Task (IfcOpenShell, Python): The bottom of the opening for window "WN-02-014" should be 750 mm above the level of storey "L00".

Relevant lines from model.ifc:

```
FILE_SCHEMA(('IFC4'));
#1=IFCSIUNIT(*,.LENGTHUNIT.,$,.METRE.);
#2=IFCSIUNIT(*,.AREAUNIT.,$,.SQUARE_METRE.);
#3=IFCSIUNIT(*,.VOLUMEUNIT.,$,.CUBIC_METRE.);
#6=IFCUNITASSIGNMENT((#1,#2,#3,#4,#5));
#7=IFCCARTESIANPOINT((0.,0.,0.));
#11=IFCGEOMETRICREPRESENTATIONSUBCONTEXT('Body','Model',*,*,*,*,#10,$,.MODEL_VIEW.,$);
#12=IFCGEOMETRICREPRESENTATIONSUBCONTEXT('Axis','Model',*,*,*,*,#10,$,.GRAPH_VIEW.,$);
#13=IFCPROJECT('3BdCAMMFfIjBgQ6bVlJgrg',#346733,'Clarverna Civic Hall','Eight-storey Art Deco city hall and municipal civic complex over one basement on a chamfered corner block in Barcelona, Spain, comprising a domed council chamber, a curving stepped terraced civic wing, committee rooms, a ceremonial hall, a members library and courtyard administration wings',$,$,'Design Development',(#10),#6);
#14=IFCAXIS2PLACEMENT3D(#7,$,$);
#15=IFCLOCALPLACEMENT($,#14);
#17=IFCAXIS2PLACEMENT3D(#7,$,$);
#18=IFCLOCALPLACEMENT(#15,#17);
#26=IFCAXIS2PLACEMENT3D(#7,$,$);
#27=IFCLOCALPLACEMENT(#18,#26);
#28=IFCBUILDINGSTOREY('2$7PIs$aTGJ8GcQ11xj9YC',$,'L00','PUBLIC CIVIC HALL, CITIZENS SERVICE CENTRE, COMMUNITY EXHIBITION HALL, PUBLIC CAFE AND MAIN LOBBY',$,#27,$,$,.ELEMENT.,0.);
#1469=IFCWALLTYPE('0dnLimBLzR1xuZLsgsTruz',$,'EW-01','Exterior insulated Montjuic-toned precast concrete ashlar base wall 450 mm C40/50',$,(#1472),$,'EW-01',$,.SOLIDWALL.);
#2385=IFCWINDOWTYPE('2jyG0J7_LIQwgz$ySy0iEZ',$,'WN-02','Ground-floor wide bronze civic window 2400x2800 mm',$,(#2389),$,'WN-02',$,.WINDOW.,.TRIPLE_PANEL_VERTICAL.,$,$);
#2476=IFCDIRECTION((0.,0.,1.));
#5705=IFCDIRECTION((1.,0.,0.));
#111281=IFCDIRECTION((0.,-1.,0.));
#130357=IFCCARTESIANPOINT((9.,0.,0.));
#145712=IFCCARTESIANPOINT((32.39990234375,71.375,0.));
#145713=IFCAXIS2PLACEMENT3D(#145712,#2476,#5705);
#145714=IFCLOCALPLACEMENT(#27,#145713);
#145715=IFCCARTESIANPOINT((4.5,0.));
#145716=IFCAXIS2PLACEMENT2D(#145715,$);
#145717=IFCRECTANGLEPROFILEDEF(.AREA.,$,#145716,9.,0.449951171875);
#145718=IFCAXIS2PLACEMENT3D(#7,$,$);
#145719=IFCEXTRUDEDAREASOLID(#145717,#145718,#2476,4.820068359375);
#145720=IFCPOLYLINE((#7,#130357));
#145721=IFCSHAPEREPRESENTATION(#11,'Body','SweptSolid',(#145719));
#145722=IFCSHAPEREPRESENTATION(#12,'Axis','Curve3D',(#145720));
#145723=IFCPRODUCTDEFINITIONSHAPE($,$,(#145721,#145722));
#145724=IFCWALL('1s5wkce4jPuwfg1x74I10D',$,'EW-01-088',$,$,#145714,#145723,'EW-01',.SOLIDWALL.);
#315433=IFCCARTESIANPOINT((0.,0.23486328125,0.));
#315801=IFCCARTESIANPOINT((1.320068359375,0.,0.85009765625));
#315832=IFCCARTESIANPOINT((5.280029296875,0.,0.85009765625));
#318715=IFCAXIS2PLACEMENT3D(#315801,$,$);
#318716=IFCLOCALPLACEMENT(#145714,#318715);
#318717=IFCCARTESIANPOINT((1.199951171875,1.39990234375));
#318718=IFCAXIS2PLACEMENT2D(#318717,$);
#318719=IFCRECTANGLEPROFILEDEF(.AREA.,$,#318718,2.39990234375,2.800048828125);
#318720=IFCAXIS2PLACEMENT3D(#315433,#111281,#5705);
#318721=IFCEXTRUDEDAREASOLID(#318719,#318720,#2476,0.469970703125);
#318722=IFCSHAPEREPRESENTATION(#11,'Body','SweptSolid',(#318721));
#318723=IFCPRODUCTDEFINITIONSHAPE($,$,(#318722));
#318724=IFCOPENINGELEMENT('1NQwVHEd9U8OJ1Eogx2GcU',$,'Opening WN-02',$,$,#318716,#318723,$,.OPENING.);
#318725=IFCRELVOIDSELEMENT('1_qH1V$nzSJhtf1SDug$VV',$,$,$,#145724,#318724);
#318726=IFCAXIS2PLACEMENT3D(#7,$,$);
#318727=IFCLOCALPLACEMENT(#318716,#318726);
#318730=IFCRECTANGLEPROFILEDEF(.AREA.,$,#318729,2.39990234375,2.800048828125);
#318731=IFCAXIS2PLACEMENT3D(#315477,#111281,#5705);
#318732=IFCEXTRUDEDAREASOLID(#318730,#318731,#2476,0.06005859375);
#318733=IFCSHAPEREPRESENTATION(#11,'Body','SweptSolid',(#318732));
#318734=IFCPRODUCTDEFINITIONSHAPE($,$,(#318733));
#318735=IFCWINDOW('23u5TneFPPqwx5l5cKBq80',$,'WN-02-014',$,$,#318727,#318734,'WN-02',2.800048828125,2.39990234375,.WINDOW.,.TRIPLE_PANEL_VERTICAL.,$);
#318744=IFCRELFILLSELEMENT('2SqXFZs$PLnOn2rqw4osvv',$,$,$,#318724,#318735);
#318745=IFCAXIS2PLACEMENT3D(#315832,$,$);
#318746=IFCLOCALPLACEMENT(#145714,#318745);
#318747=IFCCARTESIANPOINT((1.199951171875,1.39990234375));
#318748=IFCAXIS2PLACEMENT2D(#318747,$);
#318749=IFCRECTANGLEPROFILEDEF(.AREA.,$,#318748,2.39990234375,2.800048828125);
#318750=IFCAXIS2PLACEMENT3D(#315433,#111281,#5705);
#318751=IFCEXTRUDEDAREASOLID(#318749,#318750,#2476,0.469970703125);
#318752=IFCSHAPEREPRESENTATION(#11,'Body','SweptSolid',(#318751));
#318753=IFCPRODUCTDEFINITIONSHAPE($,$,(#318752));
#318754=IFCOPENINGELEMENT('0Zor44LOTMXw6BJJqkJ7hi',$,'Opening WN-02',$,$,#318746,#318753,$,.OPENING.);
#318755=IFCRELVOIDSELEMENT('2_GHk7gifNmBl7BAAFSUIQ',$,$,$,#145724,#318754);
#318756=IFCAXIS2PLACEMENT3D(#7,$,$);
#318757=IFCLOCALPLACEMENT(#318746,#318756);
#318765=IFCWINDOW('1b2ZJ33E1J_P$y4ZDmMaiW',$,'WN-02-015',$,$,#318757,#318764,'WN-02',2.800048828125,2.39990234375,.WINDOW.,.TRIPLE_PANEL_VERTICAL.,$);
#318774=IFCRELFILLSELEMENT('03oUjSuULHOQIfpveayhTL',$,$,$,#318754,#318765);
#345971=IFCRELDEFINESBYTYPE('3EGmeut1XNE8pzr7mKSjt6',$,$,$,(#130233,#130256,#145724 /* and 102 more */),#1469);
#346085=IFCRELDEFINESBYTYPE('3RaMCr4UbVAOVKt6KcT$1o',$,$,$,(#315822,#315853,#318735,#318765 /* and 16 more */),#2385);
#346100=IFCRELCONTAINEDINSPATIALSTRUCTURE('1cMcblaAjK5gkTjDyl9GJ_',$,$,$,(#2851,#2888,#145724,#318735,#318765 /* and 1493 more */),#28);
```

```python
import numpy as np
import ifcopenshell
import ifcopenshell.api.geometry
import ifcopenshell.geom
import ifcopenshell.util.element
import ifcopenshell.util.placement
import ifcopenshell.util.shape
import ifcopenshell.util.unit

model = ifcopenshell.open("model.ifc")
unit_scale = ifcopenshell.util.unit.calculate_unit_scale(model)

window = model.by_guid("23u5TneFPPqwx5l5cKBq80")
opening = window.FillsVoids[0].RelatingOpeningElement
storey = ifcopenshell.util.element.get_container(window, ifc_class="IfcBuildingStorey")
level = ifcopenshell.util.placement.get_local_placement(storey.ObjectPlacement)[2, 3]

# The opening's origin need not be at the sill, so measure its lowest point.
shape = ifcopenshell.geom.create_shape(ifcopenshell.geom.settings(), opening)
bottom = ifcopenshell.util.shape.get_shape_bottom_elevation(shape, shape.geometry) / unit_scale
dz = level + 0.75 / unit_scale - bottom

shift = np.array([0.0, 0.0, dz])
# The window is placed relative to its opening, so it follows when the opening moves.
matrix = ifcopenshell.util.placement.get_local_placement(opening.ObjectPlacement)
matrix[:3, 3] += shift
ifcopenshell.api.geometry.edit_object_placement(
    model, product=opening, matrix=matrix, is_si=False, should_transform_children=True
)

print(f"moved by {dz * unit_scale:+.3f} m")

model.write("model-out.ifc")
```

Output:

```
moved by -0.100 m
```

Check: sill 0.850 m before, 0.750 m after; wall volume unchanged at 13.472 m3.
